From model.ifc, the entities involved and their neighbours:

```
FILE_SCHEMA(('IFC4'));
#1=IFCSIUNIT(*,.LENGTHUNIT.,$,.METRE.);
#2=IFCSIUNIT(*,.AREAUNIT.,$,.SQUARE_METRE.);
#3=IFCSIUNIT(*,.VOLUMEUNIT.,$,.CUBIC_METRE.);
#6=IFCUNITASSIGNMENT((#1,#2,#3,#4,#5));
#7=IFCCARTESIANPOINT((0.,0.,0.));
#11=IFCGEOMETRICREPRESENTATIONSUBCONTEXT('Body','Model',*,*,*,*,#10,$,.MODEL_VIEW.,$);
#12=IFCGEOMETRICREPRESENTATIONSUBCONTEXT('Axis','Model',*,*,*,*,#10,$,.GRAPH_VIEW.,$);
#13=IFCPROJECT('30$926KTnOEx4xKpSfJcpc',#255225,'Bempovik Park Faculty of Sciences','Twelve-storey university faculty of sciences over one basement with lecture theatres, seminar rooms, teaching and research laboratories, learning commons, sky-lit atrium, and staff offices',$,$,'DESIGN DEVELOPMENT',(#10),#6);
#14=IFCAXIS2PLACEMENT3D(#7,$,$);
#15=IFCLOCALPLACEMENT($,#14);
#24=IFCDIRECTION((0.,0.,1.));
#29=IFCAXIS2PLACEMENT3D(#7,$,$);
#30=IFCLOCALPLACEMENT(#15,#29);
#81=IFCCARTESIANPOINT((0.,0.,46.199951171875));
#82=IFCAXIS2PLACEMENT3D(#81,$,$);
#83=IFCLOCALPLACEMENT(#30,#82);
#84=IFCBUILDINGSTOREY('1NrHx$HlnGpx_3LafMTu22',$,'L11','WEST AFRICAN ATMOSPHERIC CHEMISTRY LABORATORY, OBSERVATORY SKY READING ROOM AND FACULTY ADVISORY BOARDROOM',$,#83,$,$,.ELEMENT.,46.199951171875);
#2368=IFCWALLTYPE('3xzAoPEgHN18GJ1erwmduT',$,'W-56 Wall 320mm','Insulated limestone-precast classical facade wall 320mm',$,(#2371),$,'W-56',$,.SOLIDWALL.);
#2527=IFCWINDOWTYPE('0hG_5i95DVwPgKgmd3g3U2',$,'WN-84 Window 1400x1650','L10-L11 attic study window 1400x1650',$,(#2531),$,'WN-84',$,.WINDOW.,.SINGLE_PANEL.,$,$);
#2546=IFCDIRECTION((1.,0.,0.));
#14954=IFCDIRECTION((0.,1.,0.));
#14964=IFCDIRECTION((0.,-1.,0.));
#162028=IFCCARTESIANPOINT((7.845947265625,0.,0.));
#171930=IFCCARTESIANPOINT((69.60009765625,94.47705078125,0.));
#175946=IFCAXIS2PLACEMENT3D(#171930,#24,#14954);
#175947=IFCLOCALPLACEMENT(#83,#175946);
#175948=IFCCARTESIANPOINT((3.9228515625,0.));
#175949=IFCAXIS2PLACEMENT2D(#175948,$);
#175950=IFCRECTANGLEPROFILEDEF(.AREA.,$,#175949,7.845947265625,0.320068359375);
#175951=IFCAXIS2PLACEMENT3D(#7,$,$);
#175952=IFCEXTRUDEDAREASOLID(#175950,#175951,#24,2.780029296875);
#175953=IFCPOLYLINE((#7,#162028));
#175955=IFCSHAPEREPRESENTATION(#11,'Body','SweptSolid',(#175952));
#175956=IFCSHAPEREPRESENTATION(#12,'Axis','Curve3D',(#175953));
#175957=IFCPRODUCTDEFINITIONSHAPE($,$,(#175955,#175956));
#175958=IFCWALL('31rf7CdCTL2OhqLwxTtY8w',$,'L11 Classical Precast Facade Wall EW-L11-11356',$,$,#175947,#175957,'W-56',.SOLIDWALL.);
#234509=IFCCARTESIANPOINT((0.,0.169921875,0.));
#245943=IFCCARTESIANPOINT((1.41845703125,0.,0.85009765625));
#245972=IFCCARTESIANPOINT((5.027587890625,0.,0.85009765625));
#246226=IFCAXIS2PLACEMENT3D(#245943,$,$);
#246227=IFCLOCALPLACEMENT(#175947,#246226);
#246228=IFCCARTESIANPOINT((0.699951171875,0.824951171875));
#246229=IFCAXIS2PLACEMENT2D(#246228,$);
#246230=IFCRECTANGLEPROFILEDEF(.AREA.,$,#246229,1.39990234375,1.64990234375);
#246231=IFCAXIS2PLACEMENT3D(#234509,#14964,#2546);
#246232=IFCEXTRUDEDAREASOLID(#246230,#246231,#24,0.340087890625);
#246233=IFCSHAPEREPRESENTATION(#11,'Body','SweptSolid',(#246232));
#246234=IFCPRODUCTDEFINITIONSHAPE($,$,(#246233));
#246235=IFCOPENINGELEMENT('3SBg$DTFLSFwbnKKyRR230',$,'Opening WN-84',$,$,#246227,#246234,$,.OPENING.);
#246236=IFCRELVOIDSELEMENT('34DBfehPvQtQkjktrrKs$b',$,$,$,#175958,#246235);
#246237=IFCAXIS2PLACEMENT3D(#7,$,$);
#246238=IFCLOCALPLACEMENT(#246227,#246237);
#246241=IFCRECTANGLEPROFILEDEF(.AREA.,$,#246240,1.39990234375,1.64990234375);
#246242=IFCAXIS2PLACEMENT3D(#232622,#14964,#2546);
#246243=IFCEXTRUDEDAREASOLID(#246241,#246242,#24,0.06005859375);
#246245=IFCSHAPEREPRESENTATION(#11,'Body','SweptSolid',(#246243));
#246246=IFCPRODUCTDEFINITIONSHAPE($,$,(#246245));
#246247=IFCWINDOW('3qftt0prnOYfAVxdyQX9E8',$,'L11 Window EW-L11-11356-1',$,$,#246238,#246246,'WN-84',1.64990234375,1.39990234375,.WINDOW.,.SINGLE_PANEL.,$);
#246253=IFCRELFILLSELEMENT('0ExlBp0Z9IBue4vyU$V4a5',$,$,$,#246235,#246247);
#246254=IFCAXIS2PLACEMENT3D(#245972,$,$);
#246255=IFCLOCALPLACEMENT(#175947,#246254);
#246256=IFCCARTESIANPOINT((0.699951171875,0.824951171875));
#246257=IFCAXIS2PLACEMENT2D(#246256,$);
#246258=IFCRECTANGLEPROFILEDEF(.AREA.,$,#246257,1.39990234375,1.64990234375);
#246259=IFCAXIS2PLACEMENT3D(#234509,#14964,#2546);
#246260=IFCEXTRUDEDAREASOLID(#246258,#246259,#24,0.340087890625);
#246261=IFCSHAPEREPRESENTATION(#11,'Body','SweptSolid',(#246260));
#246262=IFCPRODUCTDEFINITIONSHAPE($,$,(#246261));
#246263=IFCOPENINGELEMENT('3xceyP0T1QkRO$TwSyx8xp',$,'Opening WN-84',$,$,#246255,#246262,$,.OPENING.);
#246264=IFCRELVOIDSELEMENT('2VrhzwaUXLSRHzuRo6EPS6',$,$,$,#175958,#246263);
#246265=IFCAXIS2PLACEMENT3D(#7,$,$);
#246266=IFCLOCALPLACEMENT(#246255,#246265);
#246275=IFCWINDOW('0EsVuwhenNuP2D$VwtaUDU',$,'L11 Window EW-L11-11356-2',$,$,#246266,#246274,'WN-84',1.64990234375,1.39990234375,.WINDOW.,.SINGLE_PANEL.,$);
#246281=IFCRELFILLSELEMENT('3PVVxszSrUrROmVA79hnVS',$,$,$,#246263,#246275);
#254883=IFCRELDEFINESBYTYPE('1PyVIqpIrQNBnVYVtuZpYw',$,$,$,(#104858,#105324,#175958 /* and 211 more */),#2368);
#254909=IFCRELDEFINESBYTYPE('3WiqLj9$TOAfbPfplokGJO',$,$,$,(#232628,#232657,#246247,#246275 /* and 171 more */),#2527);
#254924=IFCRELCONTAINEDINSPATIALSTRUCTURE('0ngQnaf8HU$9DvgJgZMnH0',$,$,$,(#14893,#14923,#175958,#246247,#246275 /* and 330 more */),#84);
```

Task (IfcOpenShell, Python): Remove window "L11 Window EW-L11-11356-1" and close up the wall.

```python
import ifcopenshell
import ifcopenshell.api.feature
import ifcopenshell.api.root
import ifcopenshell.geom
import ifcopenshell.util.shape

model = ifcopenshell.open("model.ifc")
settings = ifcopenshell.geom.settings()


def volume(element):
    """Net volume in cubic metres, openings subtracted."""
    shape = ifcopenshell.geom.create_shape(settings, element)
    return ifcopenshell.util.shape.get_volume(shape.geometry)


window = model.by_guid("3qftt0prnOYfAVxdyQX9E8")
opening = window.FillsVoids[0].RelatingOpeningElement
wall = opening.VoidsElements[0].RelatingBuildingElement
before = volume(wall)

ifcopenshell.api.root.remove_product(model, product=window)
ifcopenshell.api.feature.remove_feature(model, feature=opening)

after = volume(wall)

print(f"wall volume {before:.3f} -> {after:.3f} m3")

model.write("model_rev.ifc")
```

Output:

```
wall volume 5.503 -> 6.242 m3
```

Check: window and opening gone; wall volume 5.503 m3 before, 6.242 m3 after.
